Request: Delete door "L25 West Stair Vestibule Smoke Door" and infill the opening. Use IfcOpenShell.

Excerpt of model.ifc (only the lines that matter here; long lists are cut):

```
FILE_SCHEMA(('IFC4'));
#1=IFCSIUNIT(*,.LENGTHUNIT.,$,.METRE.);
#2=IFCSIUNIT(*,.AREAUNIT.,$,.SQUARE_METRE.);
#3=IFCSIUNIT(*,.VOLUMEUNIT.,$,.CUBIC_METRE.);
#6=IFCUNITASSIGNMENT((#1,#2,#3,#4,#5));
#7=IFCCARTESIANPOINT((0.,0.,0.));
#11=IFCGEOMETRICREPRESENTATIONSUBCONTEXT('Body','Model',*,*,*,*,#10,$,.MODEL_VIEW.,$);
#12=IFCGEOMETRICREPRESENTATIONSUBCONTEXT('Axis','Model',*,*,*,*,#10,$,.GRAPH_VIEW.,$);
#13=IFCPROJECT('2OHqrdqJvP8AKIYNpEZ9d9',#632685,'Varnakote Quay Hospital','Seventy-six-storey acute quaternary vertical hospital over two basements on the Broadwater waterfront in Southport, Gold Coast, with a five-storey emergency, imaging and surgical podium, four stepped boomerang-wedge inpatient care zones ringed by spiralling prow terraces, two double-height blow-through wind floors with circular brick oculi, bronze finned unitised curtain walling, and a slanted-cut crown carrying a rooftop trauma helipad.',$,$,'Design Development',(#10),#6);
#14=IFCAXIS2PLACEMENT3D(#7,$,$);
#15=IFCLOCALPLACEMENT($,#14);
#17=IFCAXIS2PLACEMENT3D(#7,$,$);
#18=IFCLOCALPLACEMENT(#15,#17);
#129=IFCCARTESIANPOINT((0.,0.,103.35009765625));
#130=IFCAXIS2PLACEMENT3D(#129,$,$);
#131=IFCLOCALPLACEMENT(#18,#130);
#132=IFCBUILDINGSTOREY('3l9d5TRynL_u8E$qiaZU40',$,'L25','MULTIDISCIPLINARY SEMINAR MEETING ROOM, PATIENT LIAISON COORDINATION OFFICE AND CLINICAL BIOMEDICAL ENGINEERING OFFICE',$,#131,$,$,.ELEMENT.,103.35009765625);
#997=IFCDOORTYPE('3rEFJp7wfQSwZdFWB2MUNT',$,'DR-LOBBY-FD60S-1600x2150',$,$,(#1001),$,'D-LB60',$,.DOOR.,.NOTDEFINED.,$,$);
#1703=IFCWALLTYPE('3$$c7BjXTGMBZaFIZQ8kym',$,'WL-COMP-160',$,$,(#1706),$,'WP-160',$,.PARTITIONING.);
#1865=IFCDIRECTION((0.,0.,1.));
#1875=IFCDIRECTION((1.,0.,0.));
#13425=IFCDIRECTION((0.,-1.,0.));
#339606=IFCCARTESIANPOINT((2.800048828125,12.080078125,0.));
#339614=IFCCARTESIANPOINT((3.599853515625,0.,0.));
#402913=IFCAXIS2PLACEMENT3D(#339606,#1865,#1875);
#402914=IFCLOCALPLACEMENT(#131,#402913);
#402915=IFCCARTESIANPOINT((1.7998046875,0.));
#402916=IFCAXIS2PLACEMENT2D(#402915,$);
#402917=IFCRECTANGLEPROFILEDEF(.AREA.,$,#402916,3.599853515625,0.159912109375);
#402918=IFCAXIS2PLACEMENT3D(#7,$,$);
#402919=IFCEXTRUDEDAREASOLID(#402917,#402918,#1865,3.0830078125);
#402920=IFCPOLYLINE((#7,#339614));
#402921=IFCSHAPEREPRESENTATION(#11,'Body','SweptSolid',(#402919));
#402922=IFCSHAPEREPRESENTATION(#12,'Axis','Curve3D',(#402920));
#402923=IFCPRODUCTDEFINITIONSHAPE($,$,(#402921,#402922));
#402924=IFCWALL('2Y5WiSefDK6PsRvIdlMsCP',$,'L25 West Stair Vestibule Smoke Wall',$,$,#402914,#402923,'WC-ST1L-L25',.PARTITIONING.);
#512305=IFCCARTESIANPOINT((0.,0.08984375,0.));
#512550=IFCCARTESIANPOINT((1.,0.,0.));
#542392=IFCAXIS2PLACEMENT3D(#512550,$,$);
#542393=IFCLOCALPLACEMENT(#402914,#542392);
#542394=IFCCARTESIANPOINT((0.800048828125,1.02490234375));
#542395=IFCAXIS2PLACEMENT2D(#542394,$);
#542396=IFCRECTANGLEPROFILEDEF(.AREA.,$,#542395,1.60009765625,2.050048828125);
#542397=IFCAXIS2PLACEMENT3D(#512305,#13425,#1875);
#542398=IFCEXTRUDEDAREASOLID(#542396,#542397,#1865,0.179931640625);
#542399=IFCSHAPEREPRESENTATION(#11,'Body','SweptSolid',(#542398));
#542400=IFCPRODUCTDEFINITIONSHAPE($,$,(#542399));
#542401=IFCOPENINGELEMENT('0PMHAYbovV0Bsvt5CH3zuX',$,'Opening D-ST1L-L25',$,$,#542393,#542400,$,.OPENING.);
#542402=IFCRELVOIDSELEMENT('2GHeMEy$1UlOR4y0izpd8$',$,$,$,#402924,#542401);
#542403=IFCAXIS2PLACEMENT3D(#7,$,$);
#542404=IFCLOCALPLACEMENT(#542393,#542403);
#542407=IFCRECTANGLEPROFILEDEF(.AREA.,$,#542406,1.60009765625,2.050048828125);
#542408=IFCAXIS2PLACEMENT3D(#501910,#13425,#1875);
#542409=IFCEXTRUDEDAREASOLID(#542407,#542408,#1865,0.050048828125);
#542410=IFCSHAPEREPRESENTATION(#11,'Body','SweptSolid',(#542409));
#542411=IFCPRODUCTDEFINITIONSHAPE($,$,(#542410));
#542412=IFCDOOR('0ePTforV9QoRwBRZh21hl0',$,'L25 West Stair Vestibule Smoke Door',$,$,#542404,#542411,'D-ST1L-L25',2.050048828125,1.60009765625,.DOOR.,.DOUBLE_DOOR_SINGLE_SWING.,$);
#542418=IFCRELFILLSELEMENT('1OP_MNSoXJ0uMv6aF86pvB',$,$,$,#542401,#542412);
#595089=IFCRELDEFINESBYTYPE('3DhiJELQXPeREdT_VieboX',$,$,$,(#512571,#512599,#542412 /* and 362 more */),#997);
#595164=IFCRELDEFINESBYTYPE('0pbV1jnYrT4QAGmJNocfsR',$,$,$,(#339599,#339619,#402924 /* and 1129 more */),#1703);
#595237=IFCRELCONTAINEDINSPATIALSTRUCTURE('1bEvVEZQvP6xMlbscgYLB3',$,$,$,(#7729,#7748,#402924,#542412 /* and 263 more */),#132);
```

```python
import ifcopenshell
import ifcopenshell.api.feature
import ifcopenshell.api.root
import ifcopenshell.geom
import ifcopenshell.util.shape

model = ifcopenshell.open("model.ifc")
settings = ifcopenshell.geom.settings()


def volume(element):
    """Net volume in cubic metres, openings subtracted."""
    shape = ifcopenshell.geom.create_shape(settings, element)
    return ifcopenshell.util.shape.get_volume(shape.geometry)


door = model.by_guid("0ePTforV9QoRwBRZh21hl0")
opening = door.FillsVoids[0].RelatingOpeningElement
wall = opening.VoidsElements[0].RelatingBuildingElement
before = volume(wall)

ifcopenshell.api.root.remove_product(model, product=door)
ifcopenshell.api.feature.remove_feature(model, feature=opening)

after = volume(wall)

print(f"wall volume {before:.3f} -> {after:.3f} m3")

model.write("model_rev.ifc")
```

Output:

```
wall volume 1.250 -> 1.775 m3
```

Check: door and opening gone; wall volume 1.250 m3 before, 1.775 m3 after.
